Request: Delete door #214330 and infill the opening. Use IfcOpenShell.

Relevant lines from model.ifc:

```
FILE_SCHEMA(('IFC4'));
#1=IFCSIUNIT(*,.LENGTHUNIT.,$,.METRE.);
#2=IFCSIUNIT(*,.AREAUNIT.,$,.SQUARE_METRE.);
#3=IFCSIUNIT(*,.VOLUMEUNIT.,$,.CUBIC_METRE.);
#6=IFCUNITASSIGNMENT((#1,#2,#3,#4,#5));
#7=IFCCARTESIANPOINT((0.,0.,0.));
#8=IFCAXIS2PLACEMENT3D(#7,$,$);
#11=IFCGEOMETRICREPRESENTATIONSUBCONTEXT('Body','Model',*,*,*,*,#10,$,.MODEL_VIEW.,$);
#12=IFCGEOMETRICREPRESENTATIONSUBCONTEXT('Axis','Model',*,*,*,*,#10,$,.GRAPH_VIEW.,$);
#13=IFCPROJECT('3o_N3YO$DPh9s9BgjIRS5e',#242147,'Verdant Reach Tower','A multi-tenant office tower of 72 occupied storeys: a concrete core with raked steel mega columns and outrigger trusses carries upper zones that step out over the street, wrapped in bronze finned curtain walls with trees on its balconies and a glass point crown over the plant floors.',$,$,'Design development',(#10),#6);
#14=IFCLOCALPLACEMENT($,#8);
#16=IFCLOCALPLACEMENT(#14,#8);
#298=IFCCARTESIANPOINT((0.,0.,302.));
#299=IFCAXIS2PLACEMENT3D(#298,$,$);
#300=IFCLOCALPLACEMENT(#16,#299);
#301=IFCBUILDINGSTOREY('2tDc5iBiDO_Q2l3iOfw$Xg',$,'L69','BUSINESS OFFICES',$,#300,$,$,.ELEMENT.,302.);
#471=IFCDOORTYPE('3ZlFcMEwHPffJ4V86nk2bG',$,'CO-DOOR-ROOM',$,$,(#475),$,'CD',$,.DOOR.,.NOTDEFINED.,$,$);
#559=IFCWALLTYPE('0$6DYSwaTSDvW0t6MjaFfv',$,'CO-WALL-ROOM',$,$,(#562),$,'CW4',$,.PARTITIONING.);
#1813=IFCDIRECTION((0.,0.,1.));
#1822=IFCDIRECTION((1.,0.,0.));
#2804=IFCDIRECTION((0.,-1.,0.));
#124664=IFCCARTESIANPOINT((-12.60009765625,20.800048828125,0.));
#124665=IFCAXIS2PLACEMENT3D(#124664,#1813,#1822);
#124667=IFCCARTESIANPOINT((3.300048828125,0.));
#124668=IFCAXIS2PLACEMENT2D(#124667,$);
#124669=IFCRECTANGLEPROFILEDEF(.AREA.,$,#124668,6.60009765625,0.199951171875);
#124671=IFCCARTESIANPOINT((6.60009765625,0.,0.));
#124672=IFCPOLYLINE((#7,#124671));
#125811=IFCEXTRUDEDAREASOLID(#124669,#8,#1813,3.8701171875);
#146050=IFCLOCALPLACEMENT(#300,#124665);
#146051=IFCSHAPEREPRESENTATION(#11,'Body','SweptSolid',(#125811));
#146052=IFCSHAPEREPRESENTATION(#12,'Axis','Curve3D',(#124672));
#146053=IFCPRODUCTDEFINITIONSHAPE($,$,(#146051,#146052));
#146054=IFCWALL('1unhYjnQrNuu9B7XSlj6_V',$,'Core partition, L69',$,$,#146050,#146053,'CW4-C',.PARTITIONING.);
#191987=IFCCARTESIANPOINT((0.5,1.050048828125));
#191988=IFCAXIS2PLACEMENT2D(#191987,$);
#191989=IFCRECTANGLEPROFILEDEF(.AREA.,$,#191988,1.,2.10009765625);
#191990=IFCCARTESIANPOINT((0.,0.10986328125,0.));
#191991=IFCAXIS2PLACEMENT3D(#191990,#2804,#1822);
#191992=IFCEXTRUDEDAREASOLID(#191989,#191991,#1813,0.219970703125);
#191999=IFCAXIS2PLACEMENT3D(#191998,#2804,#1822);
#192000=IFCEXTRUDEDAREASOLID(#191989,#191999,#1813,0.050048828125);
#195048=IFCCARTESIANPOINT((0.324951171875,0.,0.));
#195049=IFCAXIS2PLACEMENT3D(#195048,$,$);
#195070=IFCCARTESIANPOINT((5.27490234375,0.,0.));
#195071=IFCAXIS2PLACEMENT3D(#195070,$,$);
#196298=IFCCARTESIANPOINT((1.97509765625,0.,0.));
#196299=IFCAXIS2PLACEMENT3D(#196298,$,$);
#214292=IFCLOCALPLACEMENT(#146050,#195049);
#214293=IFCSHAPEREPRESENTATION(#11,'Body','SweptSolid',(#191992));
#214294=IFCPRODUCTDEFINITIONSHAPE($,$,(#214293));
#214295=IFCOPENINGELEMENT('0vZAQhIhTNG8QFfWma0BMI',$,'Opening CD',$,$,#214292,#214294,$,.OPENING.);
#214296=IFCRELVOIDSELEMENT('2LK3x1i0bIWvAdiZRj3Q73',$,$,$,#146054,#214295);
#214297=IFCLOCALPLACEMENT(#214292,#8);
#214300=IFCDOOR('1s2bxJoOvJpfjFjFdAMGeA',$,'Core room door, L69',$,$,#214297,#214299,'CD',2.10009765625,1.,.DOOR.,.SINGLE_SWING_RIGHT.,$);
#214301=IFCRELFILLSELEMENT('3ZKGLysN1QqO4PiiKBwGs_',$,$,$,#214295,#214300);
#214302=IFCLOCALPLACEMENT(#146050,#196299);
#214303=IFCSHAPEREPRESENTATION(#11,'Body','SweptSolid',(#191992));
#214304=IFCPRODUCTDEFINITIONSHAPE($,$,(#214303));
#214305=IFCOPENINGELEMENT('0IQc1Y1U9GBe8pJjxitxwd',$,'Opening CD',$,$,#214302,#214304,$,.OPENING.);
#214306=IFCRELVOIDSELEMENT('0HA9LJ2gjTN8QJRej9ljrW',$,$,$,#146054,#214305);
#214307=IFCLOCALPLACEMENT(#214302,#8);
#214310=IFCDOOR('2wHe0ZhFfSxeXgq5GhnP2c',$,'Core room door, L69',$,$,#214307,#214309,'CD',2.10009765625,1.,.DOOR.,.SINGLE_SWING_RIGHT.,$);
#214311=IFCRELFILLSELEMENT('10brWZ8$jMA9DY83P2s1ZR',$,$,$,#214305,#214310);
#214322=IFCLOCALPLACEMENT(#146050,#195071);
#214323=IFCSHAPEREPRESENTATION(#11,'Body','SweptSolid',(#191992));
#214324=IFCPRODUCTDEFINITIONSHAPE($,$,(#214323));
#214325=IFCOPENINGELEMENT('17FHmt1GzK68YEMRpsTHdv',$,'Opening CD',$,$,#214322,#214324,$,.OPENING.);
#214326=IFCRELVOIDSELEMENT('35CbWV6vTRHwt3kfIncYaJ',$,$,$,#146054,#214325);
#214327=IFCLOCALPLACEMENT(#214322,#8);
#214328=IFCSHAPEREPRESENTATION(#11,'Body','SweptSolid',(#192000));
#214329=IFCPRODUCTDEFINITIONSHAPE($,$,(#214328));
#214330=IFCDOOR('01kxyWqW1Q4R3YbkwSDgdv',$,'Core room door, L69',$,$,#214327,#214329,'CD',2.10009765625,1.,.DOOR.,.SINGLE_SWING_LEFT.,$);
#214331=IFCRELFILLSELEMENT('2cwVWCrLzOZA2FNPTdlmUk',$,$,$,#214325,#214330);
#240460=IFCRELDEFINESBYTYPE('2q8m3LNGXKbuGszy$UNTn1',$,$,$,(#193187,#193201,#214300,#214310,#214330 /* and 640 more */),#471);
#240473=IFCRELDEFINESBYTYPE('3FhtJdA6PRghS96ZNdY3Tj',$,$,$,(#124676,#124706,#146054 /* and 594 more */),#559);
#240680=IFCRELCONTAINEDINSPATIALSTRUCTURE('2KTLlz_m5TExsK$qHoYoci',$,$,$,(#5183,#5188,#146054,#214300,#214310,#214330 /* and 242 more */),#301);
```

```python
import ifcopenshell
import ifcopenshell.api.feature
import ifcopenshell.api.root
import ifcopenshell.geom
import ifcopenshell.util.shape

model = ifcopenshell.open("model.ifc")
settings = ifcopenshell.geom.settings()


def volume(element):
    """Net volume in cubic metres, openings subtracted."""
    shape = ifcopenshell.geom.create_shape(settings, element)
    return ifcopenshell.util.shape.get_volume(shape.geometry)


door = model.by_id(214330)
opening = door.FillsVoids[0].RelatingOpeningElement
wall = opening.VoidsElements[0].RelatingBuildingElement
before = volume(wall)

ifcopenshell.api.root.remove_product(model, product=door)
ifcopenshell.api.feature.remove_feature(model, feature=opening)

after = volume(wall)

print(f"wall volume {before:.3f} -> {after:.3f} m3")

model.write("model_updated.ifc")
```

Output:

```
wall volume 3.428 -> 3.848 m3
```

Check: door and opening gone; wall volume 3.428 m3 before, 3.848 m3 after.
